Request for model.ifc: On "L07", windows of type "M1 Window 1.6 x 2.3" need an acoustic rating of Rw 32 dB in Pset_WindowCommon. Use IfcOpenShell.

First a look at what the model holds.

```python
import ifcopenshell
import ifcopenshell.util.element

model = ifcopenshell.open("model.ifc")
print(model.schema)
storey = next(s for s in model.by_type("IfcBuildingStorey") if s.Name == "L07")
windows = [e for e in ifcopenshell.util.element.get_decomposition(storey) if e.is_a("IfcWindow")]
seen = {}
for e in windows:
    element_type = ifcopenshell.util.element.get_type(e)
    key = (element_type.Name if element_type != e and element_type else None, ifcopenshell.util.element.get_pset(e, "Pset_WindowCommon", "AcousticRating"))
    seen[key] = seen.get(key, 0) + 1
for (name, value), count in sorted(seen.items(), key=str):
    print(count, "x", name, "|", value)
```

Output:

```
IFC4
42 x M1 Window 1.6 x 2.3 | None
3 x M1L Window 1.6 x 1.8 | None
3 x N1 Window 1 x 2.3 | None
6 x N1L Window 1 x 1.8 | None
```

```python
import ifcopenshell
import ifcopenshell.api.pset
import ifcopenshell.util.element

model = ifcopenshell.open("model.ifc")

storey = next(s for s in model.by_type("IfcBuildingStorey") if s.Name == "L07")
windows = [e for e in ifcopenshell.util.element.get_decomposition(storey) if e.is_a("IfcWindow")]

count = 0
for e in windows:
    element_type = ifcopenshell.util.element.get_type(e)
    if element_type in (None, e) or element_type.Name != "M1 Window 1.6 x 2.3":
        continue
    found = ifcopenshell.util.element.get_pset(e, "Pset_WindowCommon", should_inherit=False)
    if found:
        pset = model.by_id(found["id"])
        if len(ifcopenshell.util.element.get_elements_by_pset(pset)) > 1:
            pset = ifcopenshell.api.pset.unshare_pset(model, products=[e], pset=pset)[0]
    else:
        pset = ifcopenshell.api.pset.add_pset(model, product=e, name="Pset_WindowCommon")
    ifcopenshell.api.pset.edit_pset(model, pset=pset, properties={"AcousticRating": "Rw 32 dB"})
    count += 1

print(count, "windows updated")

model.write("model_updated.ifc")
```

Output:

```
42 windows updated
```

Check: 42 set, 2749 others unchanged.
